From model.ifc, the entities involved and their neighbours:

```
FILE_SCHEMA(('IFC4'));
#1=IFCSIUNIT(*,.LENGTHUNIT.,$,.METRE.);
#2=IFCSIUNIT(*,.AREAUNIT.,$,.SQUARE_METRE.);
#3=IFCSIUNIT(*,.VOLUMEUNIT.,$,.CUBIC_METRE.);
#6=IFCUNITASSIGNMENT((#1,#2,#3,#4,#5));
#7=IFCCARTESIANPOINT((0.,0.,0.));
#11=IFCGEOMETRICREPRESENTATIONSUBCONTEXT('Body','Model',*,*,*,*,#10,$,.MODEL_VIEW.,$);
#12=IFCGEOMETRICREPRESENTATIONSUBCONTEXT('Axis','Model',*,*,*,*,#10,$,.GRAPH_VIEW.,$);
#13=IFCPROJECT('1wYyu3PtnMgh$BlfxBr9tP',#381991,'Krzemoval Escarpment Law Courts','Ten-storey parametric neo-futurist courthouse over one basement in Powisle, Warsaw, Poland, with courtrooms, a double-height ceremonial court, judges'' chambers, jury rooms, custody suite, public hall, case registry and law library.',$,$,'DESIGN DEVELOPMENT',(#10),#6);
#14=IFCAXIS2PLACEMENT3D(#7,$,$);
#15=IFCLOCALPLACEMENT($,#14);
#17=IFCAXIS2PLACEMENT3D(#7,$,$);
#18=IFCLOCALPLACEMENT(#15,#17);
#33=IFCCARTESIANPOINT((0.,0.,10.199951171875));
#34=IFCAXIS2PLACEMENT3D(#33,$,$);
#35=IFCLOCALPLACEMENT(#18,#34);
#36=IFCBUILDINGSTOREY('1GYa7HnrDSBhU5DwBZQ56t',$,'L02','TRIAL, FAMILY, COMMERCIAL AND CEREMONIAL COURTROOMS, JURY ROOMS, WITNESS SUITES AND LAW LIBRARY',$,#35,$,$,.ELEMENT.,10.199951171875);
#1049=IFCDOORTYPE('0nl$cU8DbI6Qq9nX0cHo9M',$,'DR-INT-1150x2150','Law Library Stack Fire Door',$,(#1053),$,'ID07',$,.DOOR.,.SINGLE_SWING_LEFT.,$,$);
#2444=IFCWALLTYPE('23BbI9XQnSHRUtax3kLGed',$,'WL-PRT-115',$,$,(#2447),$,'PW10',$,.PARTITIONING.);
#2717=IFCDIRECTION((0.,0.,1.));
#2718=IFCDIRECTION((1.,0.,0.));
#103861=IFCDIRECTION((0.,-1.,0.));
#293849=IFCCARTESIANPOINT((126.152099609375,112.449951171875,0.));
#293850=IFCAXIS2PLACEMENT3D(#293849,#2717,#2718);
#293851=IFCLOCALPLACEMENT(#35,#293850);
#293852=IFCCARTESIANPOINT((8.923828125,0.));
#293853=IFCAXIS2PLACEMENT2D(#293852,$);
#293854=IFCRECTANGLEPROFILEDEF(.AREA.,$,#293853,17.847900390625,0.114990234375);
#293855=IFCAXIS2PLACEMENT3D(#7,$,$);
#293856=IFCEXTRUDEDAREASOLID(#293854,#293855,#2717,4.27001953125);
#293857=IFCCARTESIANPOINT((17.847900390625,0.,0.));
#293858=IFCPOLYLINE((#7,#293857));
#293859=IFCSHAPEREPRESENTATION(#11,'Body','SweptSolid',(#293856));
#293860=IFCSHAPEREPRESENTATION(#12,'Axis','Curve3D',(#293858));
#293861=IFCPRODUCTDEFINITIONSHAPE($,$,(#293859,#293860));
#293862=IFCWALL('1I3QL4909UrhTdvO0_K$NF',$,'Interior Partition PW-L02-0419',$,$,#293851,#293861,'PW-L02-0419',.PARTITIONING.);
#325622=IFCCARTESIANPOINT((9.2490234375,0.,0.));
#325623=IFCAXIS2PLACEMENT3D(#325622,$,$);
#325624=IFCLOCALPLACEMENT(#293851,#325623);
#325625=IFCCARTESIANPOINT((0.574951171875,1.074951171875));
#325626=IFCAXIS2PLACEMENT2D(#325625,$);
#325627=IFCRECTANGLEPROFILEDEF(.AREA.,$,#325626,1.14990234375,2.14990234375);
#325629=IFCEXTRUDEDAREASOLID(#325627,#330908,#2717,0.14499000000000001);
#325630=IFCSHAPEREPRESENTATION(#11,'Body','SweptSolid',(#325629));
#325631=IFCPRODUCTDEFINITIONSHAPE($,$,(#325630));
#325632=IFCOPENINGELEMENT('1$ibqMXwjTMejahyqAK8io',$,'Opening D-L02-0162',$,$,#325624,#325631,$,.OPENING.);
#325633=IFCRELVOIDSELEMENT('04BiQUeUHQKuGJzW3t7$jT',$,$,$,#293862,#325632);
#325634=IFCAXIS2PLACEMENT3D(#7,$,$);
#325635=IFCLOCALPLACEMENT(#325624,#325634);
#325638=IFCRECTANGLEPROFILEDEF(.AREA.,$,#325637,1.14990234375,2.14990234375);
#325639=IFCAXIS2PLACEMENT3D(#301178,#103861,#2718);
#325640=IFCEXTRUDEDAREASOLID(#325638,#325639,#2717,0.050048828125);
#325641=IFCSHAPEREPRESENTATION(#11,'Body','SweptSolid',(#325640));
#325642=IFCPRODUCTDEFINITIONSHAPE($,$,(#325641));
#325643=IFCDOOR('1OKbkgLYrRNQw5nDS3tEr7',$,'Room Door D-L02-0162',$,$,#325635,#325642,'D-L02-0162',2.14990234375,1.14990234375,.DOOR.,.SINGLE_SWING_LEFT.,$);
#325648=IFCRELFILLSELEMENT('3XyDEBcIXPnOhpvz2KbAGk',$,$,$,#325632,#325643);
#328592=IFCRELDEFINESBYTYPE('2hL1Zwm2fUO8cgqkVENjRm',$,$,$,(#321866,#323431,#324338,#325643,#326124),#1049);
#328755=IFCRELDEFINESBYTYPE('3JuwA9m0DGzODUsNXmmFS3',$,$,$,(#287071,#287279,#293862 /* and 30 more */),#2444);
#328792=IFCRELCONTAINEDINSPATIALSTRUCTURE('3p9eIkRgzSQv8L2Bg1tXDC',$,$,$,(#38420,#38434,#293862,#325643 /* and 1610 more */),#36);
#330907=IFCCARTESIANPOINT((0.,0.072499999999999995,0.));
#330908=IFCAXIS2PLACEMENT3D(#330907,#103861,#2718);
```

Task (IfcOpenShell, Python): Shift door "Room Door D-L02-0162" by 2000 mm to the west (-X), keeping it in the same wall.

```python
import ifcopenshell
import ifcopenshell.api.geometry
import ifcopenshell.util.placement

model = ifcopenshell.open("model.ifc")

door = model.by_id(325643)
opening = door.FillsVoids[0].RelatingOpeningElement
wall = opening.VoidsElements[0].RelatingBuildingElement

wall_matrix = ifcopenshell.util.placement.get_local_placement(wall.ObjectPlacement)
shift = wall_matrix[:3, 0] * -2.0
before = ifcopenshell.util.placement.get_local_placement(door.ObjectPlacement)[:3, 3].copy()

# The door is placed relative to its opening, so it follows when the opening moves.
matrix = ifcopenshell.util.placement.get_local_placement(opening.ObjectPlacement)
matrix[:3, 3] += shift
ifcopenshell.api.geometry.edit_object_placement(
    model, product=opening, matrix=matrix, is_si=False, should_transform_children=True
)

after = ifcopenshell.util.placement.get_local_placement(door.ObjectPlacement)[:3, 3]
print("door moved by", (after - before).round(3) + 0.0)

model.write("model_v2.ifc")
```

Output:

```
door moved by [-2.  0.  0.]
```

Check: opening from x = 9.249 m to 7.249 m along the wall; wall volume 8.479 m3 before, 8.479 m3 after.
